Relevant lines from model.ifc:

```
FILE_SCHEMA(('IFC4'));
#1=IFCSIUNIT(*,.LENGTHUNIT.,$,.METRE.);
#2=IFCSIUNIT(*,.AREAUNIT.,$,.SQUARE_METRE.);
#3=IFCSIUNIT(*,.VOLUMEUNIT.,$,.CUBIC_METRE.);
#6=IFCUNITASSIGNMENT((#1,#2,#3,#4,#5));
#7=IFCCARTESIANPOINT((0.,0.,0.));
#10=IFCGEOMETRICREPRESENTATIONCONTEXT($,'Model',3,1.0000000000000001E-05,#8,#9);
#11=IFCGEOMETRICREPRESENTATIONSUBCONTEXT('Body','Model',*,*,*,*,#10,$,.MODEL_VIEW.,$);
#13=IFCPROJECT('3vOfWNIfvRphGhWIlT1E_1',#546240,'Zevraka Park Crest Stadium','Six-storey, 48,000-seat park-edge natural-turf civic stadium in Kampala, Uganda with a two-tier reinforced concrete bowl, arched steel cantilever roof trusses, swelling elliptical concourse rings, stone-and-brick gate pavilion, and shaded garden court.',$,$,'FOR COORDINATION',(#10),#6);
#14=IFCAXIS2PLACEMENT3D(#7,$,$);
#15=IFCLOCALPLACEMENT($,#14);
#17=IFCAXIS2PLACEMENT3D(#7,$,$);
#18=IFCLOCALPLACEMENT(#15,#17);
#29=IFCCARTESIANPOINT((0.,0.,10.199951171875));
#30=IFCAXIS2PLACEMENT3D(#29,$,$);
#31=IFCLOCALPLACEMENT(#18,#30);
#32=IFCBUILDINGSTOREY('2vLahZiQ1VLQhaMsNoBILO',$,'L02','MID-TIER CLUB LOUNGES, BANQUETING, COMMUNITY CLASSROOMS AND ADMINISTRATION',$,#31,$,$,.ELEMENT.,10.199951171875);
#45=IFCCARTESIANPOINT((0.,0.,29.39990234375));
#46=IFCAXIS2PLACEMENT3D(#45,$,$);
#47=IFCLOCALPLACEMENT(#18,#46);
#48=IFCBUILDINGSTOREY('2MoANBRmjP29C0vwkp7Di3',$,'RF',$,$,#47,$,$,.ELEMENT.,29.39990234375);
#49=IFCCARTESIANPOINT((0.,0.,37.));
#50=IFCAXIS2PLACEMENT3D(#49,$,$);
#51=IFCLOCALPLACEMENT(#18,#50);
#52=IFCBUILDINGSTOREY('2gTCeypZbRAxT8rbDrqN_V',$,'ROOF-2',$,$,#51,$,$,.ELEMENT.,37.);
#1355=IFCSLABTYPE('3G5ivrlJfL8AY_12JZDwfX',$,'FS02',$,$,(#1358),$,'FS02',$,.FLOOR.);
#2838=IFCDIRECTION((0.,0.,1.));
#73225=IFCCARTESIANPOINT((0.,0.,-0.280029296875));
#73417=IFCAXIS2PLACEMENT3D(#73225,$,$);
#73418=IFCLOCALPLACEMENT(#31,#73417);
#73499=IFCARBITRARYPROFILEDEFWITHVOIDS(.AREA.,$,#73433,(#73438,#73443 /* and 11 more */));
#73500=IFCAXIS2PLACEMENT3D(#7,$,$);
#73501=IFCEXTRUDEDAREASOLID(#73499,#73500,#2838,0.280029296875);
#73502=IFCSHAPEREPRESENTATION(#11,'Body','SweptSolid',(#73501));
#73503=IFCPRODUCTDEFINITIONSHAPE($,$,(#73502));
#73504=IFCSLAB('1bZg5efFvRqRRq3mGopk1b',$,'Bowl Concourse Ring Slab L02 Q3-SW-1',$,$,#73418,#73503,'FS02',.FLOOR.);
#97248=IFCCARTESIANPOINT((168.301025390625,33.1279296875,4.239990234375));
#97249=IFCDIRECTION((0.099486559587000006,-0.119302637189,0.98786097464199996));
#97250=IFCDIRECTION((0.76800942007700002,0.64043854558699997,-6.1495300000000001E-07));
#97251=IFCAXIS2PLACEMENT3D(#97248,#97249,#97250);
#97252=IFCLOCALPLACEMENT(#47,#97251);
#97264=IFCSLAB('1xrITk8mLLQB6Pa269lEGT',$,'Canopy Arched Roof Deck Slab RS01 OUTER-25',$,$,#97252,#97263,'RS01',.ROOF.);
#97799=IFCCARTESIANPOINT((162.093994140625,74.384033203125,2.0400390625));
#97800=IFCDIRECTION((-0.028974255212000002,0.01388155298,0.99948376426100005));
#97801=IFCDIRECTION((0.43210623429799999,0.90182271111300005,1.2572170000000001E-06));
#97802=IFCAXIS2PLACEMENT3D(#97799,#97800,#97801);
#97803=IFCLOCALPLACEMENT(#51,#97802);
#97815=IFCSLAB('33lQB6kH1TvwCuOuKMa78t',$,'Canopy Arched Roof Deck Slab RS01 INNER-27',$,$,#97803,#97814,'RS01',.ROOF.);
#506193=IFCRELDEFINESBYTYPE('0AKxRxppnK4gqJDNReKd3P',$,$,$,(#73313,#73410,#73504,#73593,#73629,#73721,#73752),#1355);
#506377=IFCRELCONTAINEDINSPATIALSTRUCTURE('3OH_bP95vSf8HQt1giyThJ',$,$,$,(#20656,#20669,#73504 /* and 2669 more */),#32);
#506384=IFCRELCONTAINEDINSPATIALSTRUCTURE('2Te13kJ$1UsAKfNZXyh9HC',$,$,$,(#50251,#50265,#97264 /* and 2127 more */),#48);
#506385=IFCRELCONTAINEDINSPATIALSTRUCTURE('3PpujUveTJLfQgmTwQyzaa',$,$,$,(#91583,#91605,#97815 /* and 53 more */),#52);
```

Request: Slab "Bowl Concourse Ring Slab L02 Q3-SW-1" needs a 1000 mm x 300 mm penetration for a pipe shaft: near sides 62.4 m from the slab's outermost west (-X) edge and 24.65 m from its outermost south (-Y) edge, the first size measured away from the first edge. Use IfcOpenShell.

```python
import numpy as np
import ifcopenshell
import ifcopenshell.api.feature
import ifcopenshell.api.geometry
import ifcopenshell.api.root
import ifcopenshell.geom
import ifcopenshell.util.placement
import ifcopenshell.util.representation
import ifcopenshell.util.shape
import ifcopenshell.util.unit

model = ifcopenshell.open("model.ifc")
unit_scale = ifcopenshell.util.unit.calculate_unit_scale(model)
settings = ifcopenshell.geom.settings()


def volume(element):
    """Net volume in cubic metres, openings subtracted."""
    shape = ifcopenshell.geom.create_shape(settings, element)
    return ifcopenshell.util.shape.get_volume(shape.geometry)


slab = model.by_guid("1bZg5efFvRqRRq3mGopk1b")
before = volume(slab)

# Extent in the slab's own axes, in metres. The edges named are its -X and -Y sides.
slab_shape = ifcopenshell.geom.create_shape(settings, slab)
vertices = ifcopenshell.util.shape.get_vertices(slab_shape.geometry)
x_min, y_min, bottom = vertices.min(axis=0)
top = vertices[:, 2].max()

opening = ifcopenshell.api.root.create_entity(model, ifc_class="IfcOpeningElement", name="Pipe shaft opening", predefined_type="OPENING")
context = ifcopenshell.util.representation.get_context(model, "Model", "Body", "MODEL_VIEW")
width, depth = 1, 0.3
outline = [(0.0, 0.0), (width, 0.0), (width, depth), (0.0, depth), (0.0, 0.0)]
# Overshoot both faces by 50 mm so the cut is clean.
shape = ifcopenshell.api.geometry.add_slab_representation(
    model, context=context, depth=top - bottom + 0.1, polyline=outline
)
ifcopenshell.api.geometry.assign_representation(model, product=opening, representation=shape)

matrix = ifcopenshell.util.placement.get_local_placement(slab.ObjectPlacement)
matrix[:, 3] = matrix @ np.append(np.array([x_min + 62.4, y_min + 24.65, bottom - 0.05]) / unit_scale, 1.0)
ifcopenshell.api.geometry.edit_object_placement(model, product=opening, matrix=matrix, is_si=False)
ifcopenshell.api.feature.add_feature(model, feature=opening, element=slab)

after = volume(slab)

print(f"slab volume {before:.3f} -> {after:.3f} m3")

model.write("model_edited.ifc")
```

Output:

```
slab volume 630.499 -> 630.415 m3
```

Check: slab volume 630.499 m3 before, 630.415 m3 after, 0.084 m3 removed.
